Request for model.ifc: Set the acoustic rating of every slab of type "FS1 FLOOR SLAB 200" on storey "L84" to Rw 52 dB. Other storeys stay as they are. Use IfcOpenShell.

First a look at what the model holds.

```python
import ifcopenshell
import ifcopenshell.util.element

model = ifcopenshell.open("model.ifc")
print(model.schema)
storey = next(s for s in model.by_type("IfcBuildingStorey") if s.Name == "L84")
slabs = [e for e in ifcopenshell.util.element.get_decomposition(storey) if e.is_a("IfcSlab")]
seen = {}
for e in slabs:
    element_type = ifcopenshell.util.element.get_type(e)
    key = (element_type.Name if element_type != e and element_type else None, ifcopenshell.util.element.get_pset(e, "Pset_SlabCommon", "AcousticRating"))
    seen[key] = seen.get(key, 0) + 1
for (name, value), count in sorted(seen.items(), key=str):
    print(count, "x", name, "|", value)
```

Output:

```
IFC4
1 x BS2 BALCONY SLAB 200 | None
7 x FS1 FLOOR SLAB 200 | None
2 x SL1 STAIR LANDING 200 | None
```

```python
import ifcopenshell
import ifcopenshell.api.pset
import ifcopenshell.util.element

model = ifcopenshell.open("model.ifc")

storey = next(s for s in model.by_type("IfcBuildingStorey") if s.Name == "L84")
slabs = [e for e in ifcopenshell.util.element.get_decomposition(storey) if e.is_a("IfcSlab")]

count = 0
for e in slabs:
    element_type = ifcopenshell.util.element.get_type(e)
    if element_type in (None, e) or element_type.Name != "FS1 FLOOR SLAB 200":
        continue
    found = ifcopenshell.util.element.get_pset(e, "Pset_SlabCommon", should_inherit=False)
    if found:
        pset = model.by_id(found["id"])
        if len(ifcopenshell.util.element.get_elements_by_pset(pset)) > 1:
            pset = ifcopenshell.api.pset.unshare_pset(model, products=[e], pset=pset)[0]
    else:
        pset = ifcopenshell.api.pset.add_pset(model, product=e, name="Pset_SlabCommon")
    ifcopenshell.api.pset.edit_pset(model, pset=pset, properties={"AcousticRating": "Rw 52 dB"})
    count += 1

print(count, "slabs updated")

model.write("model_rev.ifc")
```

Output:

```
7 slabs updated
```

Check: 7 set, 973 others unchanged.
